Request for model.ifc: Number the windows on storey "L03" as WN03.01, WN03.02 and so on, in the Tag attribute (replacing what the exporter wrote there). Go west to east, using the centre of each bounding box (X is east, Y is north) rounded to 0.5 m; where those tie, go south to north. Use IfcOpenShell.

First a look at what the model holds.

```python
import ifcopenshell
import ifcopenshell.util.element
import ifcopenshell.util.placement

model = ifcopenshell.open("model.ifc")
print(model.schema)
storey = next(s for s in model.by_type("IfcBuildingStorey") if s.Name == "L03")
windows = [e for e in ifcopenshell.util.element.get_decomposition(storey) if e.is_a("IfcWindow")]
for e in sorted(windows, key=lambda e: e.id()):
    origin = ifcopenshell.util.placement.get_local_placement(e.ObjectPlacement)[:3, 3]
    print(e.id(), e.Tag, e.Name, origin.round(2) + 0.0, sep=" | ")
```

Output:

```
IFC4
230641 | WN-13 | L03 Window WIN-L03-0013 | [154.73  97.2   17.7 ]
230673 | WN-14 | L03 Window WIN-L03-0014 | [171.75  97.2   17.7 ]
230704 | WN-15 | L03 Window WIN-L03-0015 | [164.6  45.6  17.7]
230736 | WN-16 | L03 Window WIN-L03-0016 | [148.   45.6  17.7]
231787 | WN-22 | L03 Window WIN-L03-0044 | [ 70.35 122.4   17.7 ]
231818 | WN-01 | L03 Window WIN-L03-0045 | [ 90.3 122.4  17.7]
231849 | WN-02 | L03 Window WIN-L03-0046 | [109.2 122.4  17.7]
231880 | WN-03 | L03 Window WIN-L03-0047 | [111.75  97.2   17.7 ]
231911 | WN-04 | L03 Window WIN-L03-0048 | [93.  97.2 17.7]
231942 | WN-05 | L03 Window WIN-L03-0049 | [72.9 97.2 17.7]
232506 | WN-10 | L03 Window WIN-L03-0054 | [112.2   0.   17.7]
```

```python
import ifcopenshell
import ifcopenshell.geom
import ifcopenshell.util.element
import ifcopenshell.util.shape

model = ifcopenshell.open("model.ifc")
settings = ifcopenshell.geom.settings()
settings.set("use-world-coords", True)


def centre(element):
    shape = ifcopenshell.geom.create_shape(settings, element)
    return ifcopenshell.util.shape.get_bbox_centroid(shape.geometry)


storey = next(s for s in model.by_type("IfcBuildingStorey") if s.Name == "L03")
windows = [e for e in ifcopenshell.util.element.get_decomposition(storey) if e.is_a("IfcWindow")]

# Insertion points can sit at a corner or the storey origin, so sort by the geometry (in metres).
centres = {e: centre(e) for e in windows}
windows.sort(key=lambda e: (round(centres[e][0] / 0.5), centres[e][1]))

for i, e in enumerate(windows, start=1):
    number = f"WN03.{i:02d}"
    e.Tag = number
    print(e.id(), number)

model.write("model_rev.ifc")
```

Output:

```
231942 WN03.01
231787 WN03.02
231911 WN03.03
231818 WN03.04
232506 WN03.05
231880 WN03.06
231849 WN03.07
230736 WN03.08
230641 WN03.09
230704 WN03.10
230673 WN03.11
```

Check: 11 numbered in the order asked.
